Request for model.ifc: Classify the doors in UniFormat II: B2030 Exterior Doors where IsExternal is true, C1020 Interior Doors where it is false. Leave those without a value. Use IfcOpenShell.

First a look at what the model holds.

```python
import ifcopenshell
import ifcopenshell.util.element

model = ifcopenshell.open("model.ifc")
print(model.schema)
print("classifications:", [c.Name for c in model.by_type("IfcClassification")])
values = [ifcopenshell.util.element.get_pset(e, "Pset_DoorCommon", "IsExternal") for e in model.by_type("IfcDoor")]
for value in (True, False, None):
    print("IsExternal", value, values.count(value))
```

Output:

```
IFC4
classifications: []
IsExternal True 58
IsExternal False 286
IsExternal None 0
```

```python
import ifcopenshell
import ifcopenshell.api.classification
import ifcopenshell.util.element

model = ifcopenshell.open("model.ifc")

system = ifcopenshell.api.classification.add_classification(model, classification="UniFormat II")

doors = model.by_type("IfcDoor")
external = {e: ifcopenshell.util.element.get_pset(e, "Pset_DoorCommon", "IsExternal") for e in doors}
for flag, code, name in ((True, "B2030", "Exterior Doors"), (False, "C1020", "Interior Doors")):
    products = [e for e in doors if external[e] is flag]
    ifcopenshell.api.classification.add_reference(
        model, products=products, classification=system, identification=code, name=name
    )
    print(code, len(products))

model.write("model_rev.ifc")
```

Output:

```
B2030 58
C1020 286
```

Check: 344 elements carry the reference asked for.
